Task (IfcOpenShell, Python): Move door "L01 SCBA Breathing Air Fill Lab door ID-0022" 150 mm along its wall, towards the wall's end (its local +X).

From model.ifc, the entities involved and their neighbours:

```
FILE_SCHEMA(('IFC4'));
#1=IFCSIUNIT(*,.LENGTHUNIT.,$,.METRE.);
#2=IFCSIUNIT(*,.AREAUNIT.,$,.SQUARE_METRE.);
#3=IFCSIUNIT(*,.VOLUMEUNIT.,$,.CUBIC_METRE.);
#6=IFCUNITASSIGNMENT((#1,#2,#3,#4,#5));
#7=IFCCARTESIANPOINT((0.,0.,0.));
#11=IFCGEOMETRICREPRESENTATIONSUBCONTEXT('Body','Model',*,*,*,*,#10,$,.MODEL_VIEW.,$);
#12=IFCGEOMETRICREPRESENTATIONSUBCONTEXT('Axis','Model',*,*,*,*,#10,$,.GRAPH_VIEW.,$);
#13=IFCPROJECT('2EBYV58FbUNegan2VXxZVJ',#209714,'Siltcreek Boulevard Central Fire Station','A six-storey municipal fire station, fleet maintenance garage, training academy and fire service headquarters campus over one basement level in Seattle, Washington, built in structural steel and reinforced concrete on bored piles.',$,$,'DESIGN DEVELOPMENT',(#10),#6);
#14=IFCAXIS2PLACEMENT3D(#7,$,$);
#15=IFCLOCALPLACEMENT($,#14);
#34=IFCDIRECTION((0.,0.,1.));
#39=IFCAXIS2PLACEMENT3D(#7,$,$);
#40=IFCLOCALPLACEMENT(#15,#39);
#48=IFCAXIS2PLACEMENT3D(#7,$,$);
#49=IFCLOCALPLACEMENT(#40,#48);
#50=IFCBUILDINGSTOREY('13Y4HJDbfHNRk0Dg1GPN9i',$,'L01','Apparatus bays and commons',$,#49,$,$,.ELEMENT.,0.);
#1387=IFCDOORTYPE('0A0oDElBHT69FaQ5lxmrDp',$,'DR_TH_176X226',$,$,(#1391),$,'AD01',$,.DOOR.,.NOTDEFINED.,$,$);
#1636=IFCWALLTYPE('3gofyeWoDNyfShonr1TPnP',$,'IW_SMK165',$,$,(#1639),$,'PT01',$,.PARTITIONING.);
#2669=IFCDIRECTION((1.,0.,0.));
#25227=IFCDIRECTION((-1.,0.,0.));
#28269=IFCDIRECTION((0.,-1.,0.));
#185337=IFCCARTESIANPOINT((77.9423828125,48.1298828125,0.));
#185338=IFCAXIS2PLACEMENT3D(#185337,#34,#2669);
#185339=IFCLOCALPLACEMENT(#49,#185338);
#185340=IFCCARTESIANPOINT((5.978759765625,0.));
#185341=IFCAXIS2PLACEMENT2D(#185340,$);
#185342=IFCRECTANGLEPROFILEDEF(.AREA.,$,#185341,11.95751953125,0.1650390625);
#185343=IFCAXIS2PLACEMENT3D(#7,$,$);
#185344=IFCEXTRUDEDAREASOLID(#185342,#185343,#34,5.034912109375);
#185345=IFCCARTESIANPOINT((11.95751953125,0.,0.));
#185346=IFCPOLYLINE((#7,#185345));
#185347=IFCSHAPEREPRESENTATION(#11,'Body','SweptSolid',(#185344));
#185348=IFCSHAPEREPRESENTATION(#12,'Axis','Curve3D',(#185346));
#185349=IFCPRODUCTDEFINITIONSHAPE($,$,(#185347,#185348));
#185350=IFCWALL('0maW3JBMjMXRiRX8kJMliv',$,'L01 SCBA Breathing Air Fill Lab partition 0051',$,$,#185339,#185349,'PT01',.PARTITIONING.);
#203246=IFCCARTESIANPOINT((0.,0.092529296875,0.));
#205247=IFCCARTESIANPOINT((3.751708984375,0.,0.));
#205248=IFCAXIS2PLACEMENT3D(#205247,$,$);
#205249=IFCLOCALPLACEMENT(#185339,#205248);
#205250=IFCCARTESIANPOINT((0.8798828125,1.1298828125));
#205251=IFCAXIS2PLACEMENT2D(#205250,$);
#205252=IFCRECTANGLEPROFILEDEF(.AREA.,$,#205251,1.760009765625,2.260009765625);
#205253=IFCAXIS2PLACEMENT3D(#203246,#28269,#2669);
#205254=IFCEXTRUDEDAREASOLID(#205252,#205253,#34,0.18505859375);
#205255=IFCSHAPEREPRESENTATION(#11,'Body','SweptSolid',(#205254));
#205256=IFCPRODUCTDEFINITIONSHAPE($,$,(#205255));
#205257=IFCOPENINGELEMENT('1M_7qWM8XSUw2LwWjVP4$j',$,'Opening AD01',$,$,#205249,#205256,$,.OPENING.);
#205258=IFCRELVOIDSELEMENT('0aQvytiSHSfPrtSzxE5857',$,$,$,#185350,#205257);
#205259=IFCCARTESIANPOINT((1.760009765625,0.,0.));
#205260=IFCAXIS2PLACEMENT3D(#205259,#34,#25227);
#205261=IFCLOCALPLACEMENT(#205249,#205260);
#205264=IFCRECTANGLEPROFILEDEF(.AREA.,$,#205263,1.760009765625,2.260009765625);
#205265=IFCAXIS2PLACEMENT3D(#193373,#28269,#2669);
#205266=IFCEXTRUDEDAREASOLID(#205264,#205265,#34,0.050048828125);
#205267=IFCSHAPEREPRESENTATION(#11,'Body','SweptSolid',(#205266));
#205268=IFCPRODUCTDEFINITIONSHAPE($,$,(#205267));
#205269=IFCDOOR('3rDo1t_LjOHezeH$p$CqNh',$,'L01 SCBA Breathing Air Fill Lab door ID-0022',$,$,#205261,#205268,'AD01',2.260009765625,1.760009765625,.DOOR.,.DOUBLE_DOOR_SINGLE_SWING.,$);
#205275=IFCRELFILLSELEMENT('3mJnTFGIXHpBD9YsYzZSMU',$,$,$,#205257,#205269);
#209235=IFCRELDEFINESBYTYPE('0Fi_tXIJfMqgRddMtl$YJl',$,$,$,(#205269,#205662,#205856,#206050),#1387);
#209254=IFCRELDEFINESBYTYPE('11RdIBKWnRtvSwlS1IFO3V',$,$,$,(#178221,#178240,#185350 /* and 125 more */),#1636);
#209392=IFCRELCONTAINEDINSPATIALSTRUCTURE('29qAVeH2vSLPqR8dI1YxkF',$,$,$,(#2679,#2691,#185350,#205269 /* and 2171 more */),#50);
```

```python
import ifcopenshell
import ifcopenshell.api.geometry
import ifcopenshell.util.placement

model = ifcopenshell.open("model.ifc")

door = model.by_guid("3rDo1t_LjOHezeH$p$CqNh")
opening = door.FillsVoids[0].RelatingOpeningElement
wall = opening.VoidsElements[0].RelatingBuildingElement

wall_matrix = ifcopenshell.util.placement.get_local_placement(wall.ObjectPlacement)
shift = wall_matrix[:3, 0] * 0.15
before = ifcopenshell.util.placement.get_local_placement(door.ObjectPlacement)[:3, 3].copy()

# The door is placed relative to its opening, so it follows when the opening moves.
matrix = ifcopenshell.util.placement.get_local_placement(opening.ObjectPlacement)
matrix[:3, 3] += shift
ifcopenshell.api.geometry.edit_object_placement(
    model, product=opening, matrix=matrix, is_si=False, should_transform_children=True
)

after = ifcopenshell.util.placement.get_local_placement(door.ObjectPlacement)[:3, 3]
print("door moved by", (after - before).round(3) + 0.0)

model.write("model_updated.ifc")
```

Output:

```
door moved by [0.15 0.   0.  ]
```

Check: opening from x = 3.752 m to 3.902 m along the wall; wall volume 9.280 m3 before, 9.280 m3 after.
